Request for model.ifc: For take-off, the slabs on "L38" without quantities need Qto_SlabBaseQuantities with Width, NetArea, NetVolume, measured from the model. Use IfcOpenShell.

First a look at what the model holds.

```python
import ifcopenshell
import ifcopenshell.util.element
import ifcopenshell.util.unit

model = ifcopenshell.open("model.ifc")
print(model.schema)
for unit_type in ("LENGTHUNIT", "AREAUNIT", "VOLUMEUNIT"):
    print(unit_type, ifcopenshell.util.unit.calculate_unit_scale(model, unit_type))
storey = next(s for s in model.by_type("IfcBuildingStorey") if s.Name == "L38")
slabs = [e for e in ifcopenshell.util.element.get_decomposition(storey) if e.is_a("IfcSlab")]
for e in sorted(slabs, key=lambda e: e.id()):
    print(e.id(), e.is_a(), e.Name, list(ifcopenshell.util.element.get_psets(e, qtos_only=True)), sep=" | ")
```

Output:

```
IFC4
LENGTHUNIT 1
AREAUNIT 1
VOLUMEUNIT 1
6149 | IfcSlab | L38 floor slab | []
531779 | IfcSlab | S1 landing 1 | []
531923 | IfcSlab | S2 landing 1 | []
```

```python
import ifcopenshell
import ifcopenshell.api.pset
import ifcopenshell.geom
import ifcopenshell.util.element
import ifcopenshell.util.shape
import ifcopenshell.util.unit

model = ifcopenshell.open("model.ifc")
unit_scale = ifcopenshell.util.unit.calculate_unit_scale(model)
area_scale = ifcopenshell.util.unit.calculate_unit_scale(model, "AREAUNIT")
volume_scale = ifcopenshell.util.unit.calculate_unit_scale(model, "VOLUMEUNIT")
settings = ifcopenshell.geom.settings()

storey = next(s for s in model.by_type("IfcBuildingStorey") if s.Name == "L38")
slabs = [e for e in ifcopenshell.util.element.get_decomposition(storey) if e.is_a("IfcSlab")]

for e in sorted(slabs, key=lambda e: e.id()):
    if ifcopenshell.util.element.get_psets(e, qtos_only=True, should_inherit=False):
        continue
    # Geometry comes back in metres, in the element's own axes.
    shape = ifcopenshell.geom.create_shape(settings, e)
    values = {
        "Width": ifcopenshell.util.shape.get_z(shape.geometry) / unit_scale,
        "NetArea": ifcopenshell.util.shape.get_footprint_area(shape.geometry) / area_scale,
        "NetVolume": ifcopenshell.util.shape.get_volume(shape.geometry) / volume_scale,
    }
    qto = ifcopenshell.api.pset.add_qto(model, product=e, name="Qto_SlabBaseQuantities")
    ifcopenshell.api.pset.edit_qto(model, qto=qto, properties=values)
    print(e.id(), {k: round(v, 3) for k, v in values.items()})

model.write("model_rev.ifc")
```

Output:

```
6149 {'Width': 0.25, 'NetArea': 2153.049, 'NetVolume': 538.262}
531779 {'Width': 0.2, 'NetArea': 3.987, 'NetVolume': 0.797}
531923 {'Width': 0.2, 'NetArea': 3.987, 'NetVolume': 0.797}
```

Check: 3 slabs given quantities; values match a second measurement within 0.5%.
